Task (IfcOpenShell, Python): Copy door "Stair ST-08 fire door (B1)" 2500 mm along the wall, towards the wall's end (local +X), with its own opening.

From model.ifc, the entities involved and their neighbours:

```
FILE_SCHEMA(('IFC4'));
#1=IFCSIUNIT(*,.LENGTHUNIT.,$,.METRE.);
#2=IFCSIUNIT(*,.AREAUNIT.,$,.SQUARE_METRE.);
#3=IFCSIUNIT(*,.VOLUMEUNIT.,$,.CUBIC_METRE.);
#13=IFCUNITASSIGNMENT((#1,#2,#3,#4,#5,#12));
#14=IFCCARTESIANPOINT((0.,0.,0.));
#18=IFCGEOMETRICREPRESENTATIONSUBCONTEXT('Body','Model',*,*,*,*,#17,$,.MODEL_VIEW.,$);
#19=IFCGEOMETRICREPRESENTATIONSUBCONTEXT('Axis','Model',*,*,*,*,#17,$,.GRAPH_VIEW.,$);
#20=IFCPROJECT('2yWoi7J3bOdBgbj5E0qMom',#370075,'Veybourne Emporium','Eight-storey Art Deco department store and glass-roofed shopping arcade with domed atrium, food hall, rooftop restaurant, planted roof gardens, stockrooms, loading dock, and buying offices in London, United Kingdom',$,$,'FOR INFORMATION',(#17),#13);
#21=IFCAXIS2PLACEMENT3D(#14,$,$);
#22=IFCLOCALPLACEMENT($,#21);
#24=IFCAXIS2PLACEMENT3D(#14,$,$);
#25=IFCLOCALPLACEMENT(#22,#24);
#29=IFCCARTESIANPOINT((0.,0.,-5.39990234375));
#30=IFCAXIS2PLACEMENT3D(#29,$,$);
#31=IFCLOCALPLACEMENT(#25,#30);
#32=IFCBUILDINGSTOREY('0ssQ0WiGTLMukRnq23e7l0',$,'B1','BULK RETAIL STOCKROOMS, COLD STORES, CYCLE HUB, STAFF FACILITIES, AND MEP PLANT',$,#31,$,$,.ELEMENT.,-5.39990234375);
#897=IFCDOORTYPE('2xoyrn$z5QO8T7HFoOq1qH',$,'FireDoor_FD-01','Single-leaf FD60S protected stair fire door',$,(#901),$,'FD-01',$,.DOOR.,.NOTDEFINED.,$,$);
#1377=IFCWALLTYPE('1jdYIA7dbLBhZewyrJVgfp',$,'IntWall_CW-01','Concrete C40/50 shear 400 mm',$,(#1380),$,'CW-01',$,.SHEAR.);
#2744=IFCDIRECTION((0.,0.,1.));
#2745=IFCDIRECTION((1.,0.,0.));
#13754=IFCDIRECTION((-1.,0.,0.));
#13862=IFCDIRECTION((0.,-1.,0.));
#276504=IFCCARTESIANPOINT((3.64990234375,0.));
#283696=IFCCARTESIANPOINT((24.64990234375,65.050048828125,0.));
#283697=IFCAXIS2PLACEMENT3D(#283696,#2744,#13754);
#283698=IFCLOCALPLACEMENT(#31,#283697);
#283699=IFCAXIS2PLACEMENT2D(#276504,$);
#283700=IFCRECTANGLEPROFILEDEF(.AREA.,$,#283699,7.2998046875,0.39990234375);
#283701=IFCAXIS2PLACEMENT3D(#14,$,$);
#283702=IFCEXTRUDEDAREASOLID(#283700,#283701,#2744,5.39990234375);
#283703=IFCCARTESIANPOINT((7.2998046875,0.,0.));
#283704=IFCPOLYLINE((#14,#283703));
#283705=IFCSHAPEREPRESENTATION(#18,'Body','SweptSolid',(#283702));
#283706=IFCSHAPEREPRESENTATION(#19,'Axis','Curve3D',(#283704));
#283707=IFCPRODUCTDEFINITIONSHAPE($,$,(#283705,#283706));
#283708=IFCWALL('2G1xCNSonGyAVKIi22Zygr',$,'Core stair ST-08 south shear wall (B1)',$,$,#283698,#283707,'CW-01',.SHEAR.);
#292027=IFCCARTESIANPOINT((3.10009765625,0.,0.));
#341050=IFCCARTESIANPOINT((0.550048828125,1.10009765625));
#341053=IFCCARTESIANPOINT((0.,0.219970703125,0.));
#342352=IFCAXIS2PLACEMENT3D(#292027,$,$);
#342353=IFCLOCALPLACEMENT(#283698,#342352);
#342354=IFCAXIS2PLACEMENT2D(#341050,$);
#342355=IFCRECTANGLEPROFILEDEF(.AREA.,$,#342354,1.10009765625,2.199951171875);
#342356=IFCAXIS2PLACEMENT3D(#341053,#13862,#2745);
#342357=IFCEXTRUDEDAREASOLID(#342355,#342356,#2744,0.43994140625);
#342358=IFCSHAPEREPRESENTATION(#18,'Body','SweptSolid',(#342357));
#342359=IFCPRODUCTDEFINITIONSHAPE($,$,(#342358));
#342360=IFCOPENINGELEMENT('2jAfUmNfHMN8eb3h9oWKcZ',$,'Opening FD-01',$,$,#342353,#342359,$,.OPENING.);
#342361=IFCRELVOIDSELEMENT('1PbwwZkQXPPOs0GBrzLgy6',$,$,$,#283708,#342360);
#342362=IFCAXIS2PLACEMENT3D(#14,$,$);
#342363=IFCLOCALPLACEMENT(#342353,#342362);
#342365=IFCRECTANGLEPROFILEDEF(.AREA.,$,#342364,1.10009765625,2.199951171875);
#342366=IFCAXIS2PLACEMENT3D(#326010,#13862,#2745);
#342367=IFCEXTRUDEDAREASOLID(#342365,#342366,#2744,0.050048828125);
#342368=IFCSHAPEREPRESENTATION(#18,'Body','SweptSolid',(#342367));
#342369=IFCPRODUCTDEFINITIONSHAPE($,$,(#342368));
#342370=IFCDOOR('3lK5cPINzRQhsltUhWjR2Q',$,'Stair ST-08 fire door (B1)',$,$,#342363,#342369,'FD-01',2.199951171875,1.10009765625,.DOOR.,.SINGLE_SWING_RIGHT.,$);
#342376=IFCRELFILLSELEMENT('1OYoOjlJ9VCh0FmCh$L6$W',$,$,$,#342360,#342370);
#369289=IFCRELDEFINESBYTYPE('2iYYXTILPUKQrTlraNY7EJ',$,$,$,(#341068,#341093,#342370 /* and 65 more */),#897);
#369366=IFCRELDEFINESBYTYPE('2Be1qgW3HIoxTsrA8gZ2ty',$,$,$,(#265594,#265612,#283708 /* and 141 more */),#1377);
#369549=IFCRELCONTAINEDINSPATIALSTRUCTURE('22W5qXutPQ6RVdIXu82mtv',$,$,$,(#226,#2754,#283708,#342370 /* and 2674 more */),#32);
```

```python
import ifcopenshell
import ifcopenshell.api.feature
import ifcopenshell.api.geometry
import ifcopenshell.api.root
import ifcopenshell.geom
import ifcopenshell.util.element
import ifcopenshell.util.placement
import ifcopenshell.util.shape
import ifcopenshell.util.unit

model = ifcopenshell.open("model.ifc")
unit_scale = ifcopenshell.util.unit.calculate_unit_scale(model)
settings = ifcopenshell.geom.settings()


def volume(element):
    """Net volume in cubic metres, openings subtracted."""
    shape = ifcopenshell.geom.create_shape(settings, element)
    return ifcopenshell.util.shape.get_volume(shape.geometry)


door = model.by_guid("3lK5cPINzRQhsltUhWjR2Q")
opening = door.FillsVoids[0].RelatingOpeningElement
wall = opening.VoidsElements[0].RelatingBuildingElement
before = volume(wall)
shift = ifcopenshell.util.placement.get_local_placement(wall.ObjectPlacement)[:3, 0] * 2.5 / unit_scale

# copy_class copies the void relationship, type, container and properties, but no geometry.
new_opening = ifcopenshell.api.root.copy_class(model, product=opening)
new_opening.Representation = ifcopenshell.util.element.copy_deep(
    model, opening.Representation, exclude=["IfcGeometricRepresentationContext", "IfcRepresentationMap"]
)
new_door = ifcopenshell.api.root.copy_class(model, product=door)
new_door.Representation = ifcopenshell.util.element.copy_deep(
    model, door.Representation, exclude=["IfcGeometricRepresentationContext", "IfcRepresentationMap"]
)
new_door.Tag = None
ifcopenshell.api.feature.add_filling(model, opening=new_opening, element=new_door)

for old, new in ((opening, new_opening), (door, new_door)):
    matrix = ifcopenshell.util.placement.get_local_placement(old.ObjectPlacement)
    matrix[:3, 3] += shift
    ifcopenshell.api.geometry.edit_object_placement(model, product=new, matrix=matrix, is_si=False)

after = volume(wall)

print(f"wall volume {before:.3f} -> {after:.3f} m3")

model.write("model_edited.ifc")
```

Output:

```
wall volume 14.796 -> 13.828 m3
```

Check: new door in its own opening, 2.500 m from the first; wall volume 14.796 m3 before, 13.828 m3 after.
